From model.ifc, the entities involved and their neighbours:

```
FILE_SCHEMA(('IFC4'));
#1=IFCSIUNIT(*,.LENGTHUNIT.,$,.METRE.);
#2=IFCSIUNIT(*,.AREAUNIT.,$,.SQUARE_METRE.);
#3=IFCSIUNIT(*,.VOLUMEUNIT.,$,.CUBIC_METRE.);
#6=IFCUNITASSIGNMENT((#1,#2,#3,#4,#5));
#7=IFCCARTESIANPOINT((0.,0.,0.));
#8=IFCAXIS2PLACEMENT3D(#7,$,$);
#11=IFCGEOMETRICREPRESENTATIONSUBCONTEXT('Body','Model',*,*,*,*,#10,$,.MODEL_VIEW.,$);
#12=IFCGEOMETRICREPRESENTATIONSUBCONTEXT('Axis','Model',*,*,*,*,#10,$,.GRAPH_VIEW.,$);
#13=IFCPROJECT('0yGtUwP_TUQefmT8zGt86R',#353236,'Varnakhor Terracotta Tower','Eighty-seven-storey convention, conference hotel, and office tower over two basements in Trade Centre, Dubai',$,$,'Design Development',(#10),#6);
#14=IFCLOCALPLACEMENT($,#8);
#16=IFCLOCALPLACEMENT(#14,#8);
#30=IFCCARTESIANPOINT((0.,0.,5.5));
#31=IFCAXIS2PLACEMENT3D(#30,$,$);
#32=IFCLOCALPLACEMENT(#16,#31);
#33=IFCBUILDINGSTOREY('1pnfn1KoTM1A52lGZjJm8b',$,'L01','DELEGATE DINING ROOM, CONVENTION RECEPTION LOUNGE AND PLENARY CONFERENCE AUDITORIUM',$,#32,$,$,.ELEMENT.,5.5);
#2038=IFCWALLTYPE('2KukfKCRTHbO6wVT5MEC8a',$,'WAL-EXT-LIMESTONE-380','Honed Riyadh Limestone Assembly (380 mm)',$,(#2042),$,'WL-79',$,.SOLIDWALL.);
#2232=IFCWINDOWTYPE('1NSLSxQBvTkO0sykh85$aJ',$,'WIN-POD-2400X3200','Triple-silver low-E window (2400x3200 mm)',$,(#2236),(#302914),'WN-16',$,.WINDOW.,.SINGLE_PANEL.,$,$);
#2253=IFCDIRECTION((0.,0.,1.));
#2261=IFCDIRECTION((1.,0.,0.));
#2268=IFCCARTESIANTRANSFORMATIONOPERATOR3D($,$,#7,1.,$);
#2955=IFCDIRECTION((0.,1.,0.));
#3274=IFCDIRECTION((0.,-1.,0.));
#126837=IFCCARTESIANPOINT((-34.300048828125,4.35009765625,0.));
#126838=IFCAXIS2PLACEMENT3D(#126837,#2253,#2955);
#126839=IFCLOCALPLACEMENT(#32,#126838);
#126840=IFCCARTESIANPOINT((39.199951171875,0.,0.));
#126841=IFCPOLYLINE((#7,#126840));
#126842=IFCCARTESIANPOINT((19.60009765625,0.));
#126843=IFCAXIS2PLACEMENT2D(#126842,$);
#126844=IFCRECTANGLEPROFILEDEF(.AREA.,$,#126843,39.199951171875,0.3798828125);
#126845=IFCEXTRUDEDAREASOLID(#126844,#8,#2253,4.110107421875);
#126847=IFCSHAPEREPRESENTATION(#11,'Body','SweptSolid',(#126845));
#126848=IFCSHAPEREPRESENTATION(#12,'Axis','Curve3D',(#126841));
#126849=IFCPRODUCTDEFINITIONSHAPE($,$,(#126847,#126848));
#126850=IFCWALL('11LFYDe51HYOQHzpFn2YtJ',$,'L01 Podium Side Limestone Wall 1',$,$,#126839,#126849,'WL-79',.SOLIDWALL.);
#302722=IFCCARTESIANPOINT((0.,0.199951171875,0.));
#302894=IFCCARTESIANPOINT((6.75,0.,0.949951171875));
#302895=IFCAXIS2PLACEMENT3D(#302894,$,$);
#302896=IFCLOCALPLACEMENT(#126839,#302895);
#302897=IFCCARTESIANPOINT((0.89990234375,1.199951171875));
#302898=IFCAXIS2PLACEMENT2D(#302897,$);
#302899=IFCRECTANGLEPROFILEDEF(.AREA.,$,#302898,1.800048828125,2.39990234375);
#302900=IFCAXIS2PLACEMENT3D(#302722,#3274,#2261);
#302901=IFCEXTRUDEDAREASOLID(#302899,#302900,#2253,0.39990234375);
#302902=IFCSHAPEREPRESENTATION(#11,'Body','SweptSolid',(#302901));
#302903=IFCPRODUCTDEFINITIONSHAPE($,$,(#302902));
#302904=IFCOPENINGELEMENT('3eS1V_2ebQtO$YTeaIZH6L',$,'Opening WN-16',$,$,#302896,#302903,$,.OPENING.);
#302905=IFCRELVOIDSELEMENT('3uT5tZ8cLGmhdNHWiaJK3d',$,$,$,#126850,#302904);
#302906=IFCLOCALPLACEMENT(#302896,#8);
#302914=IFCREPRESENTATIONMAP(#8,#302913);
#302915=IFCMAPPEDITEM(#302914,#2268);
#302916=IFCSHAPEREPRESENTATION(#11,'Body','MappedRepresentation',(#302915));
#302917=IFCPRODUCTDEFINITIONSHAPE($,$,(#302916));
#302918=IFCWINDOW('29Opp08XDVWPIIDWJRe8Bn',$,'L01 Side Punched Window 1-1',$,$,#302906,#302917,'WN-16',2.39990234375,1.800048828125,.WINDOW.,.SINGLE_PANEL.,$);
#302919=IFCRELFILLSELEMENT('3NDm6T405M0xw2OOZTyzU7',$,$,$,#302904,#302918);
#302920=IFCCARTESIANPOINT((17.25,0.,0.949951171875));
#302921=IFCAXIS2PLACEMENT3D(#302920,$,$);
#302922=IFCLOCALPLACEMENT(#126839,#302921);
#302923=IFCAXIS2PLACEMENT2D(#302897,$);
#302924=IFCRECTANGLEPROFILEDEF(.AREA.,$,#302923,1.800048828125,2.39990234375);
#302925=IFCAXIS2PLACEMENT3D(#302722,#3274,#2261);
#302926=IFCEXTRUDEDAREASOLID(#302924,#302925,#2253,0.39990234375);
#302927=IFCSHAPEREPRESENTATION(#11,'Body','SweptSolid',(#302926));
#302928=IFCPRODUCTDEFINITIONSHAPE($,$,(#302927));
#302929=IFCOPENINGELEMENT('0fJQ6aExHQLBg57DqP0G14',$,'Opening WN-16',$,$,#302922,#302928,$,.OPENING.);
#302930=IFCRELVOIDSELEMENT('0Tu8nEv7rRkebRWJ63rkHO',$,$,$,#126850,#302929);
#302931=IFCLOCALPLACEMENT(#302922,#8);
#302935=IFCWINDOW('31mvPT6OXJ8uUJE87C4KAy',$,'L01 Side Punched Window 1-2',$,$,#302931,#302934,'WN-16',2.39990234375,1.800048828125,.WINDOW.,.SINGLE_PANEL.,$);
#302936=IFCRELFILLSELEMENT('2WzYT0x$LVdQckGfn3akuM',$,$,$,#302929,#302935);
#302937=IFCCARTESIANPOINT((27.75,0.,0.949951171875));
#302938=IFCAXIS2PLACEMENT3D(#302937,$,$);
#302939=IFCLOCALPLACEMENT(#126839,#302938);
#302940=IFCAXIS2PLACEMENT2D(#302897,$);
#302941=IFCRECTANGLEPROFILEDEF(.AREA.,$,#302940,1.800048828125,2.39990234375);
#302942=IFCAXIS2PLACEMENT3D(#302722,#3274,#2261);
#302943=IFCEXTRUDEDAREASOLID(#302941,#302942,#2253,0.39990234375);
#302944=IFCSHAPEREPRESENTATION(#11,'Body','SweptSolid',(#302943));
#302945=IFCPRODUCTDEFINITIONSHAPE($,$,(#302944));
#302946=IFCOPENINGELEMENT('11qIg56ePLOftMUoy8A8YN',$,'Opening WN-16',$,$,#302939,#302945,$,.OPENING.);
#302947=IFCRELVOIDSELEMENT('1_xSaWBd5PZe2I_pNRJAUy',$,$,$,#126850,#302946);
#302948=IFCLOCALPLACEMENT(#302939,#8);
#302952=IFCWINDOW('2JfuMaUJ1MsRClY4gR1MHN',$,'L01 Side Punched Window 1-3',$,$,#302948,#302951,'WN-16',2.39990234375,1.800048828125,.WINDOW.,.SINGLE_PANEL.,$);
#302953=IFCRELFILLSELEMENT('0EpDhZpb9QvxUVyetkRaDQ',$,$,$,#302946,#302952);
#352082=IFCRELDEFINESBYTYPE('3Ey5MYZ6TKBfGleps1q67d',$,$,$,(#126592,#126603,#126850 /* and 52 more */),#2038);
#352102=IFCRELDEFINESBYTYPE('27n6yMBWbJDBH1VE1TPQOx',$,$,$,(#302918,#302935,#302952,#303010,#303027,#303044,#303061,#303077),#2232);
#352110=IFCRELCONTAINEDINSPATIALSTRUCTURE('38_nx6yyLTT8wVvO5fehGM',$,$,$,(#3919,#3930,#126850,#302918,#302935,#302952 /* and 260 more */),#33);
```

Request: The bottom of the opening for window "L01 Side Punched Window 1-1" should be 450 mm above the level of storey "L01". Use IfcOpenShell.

```python
import numpy as np
import ifcopenshell
import ifcopenshell.api.geometry
import ifcopenshell.geom
import ifcopenshell.util.element
import ifcopenshell.util.placement
import ifcopenshell.util.shape
import ifcopenshell.util.unit

model = ifcopenshell.open("model.ifc")
unit_scale = ifcopenshell.util.unit.calculate_unit_scale(model)

window = model.by_guid("29Opp08XDVWPIIDWJRe8Bn")
opening = window.FillsVoids[0].RelatingOpeningElement
storey = ifcopenshell.util.element.get_container(window, ifc_class="IfcBuildingStorey")
level = ifcopenshell.util.placement.get_local_placement(storey.ObjectPlacement)[2, 3]

# The opening's origin need not be at the sill, so measure its lowest point.
shape = ifcopenshell.geom.create_shape(ifcopenshell.geom.settings(), opening)
bottom = ifcopenshell.util.shape.get_shape_bottom_elevation(shape, shape.geometry) / unit_scale
dz = level + 0.45 / unit_scale - bottom

shift = np.array([0.0, 0.0, dz])
# The window is placed relative to its opening, so it follows when the opening moves.
matrix = ifcopenshell.util.placement.get_local_placement(opening.ObjectPlacement)
matrix[:3, 3] += shift
ifcopenshell.api.geometry.edit_object_placement(
    model, product=opening, matrix=matrix, is_si=False, should_transform_children=True
)

print(f"moved by {dz * unit_scale:+.3f} m")

model.write("model_rev.ifc")
```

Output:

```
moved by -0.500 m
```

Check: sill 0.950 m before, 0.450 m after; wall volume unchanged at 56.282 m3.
